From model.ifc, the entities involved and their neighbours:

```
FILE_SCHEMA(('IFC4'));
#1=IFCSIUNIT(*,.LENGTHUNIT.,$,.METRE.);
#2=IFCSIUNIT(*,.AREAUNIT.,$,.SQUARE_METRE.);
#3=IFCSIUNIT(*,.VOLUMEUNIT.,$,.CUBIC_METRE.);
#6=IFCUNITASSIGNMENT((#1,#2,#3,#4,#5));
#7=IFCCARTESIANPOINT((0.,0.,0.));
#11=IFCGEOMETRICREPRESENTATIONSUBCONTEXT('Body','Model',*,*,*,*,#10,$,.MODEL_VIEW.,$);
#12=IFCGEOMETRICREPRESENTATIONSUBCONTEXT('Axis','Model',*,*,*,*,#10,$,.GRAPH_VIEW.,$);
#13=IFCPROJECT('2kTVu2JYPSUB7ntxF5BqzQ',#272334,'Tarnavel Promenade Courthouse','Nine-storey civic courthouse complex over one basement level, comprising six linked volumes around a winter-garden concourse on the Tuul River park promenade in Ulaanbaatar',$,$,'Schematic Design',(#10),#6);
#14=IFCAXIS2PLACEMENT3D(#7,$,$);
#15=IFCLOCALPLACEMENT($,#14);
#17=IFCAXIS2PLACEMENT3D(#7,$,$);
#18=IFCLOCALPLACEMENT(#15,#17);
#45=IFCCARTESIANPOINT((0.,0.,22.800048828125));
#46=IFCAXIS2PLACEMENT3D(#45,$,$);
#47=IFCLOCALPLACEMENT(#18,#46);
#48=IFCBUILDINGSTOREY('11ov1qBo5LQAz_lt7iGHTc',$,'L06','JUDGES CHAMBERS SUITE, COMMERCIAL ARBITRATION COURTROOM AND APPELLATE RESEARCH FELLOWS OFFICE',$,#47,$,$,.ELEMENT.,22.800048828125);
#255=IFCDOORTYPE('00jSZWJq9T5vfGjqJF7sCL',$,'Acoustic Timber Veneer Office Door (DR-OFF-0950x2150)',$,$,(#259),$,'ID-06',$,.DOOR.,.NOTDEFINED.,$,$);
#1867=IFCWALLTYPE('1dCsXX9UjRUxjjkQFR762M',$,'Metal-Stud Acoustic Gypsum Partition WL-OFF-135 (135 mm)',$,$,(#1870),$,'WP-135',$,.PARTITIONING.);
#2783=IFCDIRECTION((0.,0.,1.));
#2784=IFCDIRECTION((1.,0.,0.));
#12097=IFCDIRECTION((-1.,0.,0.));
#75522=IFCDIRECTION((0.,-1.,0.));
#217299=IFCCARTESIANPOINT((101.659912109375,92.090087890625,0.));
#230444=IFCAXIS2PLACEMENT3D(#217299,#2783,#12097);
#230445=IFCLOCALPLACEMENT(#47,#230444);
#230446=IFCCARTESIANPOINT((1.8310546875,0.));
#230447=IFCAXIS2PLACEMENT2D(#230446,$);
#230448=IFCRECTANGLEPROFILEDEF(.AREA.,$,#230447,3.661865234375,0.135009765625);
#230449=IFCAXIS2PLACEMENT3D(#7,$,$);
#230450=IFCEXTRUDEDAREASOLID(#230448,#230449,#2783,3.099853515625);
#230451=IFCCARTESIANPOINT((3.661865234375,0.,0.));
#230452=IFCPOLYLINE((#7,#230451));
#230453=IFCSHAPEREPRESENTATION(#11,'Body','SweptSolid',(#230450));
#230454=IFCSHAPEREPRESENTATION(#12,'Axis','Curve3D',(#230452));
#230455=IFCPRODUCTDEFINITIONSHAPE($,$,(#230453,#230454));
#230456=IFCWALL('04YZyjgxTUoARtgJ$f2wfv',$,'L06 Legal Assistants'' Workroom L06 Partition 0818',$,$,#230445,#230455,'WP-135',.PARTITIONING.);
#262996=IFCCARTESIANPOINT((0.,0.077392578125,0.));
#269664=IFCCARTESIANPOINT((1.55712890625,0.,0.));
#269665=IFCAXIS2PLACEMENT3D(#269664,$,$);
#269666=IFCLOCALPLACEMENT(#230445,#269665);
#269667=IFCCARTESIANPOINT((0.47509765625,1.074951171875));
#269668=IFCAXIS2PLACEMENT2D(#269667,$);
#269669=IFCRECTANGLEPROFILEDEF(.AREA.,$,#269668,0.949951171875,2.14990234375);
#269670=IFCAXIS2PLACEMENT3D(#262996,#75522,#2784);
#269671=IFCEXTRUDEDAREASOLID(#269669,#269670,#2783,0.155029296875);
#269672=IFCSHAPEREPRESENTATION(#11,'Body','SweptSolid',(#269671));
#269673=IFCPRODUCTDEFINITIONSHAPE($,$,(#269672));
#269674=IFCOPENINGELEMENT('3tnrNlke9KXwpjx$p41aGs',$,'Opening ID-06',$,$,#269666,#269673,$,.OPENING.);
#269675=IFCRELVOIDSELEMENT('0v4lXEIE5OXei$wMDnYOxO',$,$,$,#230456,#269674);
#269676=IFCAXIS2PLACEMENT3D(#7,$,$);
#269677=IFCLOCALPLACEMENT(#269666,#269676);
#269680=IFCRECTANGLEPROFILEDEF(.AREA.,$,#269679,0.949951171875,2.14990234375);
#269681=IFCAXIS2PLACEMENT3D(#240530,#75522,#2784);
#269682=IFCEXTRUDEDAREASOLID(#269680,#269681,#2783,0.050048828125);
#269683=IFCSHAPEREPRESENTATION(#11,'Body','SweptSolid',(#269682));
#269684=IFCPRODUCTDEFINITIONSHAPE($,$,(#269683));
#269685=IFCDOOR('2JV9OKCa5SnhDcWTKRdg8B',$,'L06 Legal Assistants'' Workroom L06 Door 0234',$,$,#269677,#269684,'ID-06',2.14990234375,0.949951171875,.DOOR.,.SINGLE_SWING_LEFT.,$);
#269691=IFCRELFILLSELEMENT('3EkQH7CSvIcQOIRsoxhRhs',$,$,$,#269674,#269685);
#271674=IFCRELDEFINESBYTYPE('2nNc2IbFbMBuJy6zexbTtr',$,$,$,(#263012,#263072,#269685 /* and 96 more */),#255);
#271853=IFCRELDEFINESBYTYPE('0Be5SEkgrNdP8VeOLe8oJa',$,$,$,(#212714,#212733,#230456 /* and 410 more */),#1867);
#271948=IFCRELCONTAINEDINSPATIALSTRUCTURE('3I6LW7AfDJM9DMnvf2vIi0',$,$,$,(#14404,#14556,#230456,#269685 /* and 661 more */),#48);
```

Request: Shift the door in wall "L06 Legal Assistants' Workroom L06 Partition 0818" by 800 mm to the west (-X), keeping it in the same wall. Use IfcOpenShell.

```python
import ifcopenshell
import ifcopenshell.api.geometry
import ifcopenshell.util.placement

model = ifcopenshell.open("model.ifc")

door = model.by_guid("2JV9OKCa5SnhDcWTKRdg8B")
opening = door.FillsVoids[0].RelatingOpeningElement
wall = opening.VoidsElements[0].RelatingBuildingElement

wall_matrix = ifcopenshell.util.placement.get_local_placement(wall.ObjectPlacement)
shift = wall_matrix[:3, 0] * 0.8
before = ifcopenshell.util.placement.get_local_placement(door.ObjectPlacement)[:3, 3].copy()

# The door is placed relative to its opening, so it follows when the opening moves.
matrix = ifcopenshell.util.placement.get_local_placement(opening.ObjectPlacement)
matrix[:3, 3] += shift
ifcopenshell.api.geometry.edit_object_placement(
    model, product=opening, matrix=matrix, is_si=False, should_transform_children=True
)

after = ifcopenshell.util.placement.get_local_placement(door.ObjectPlacement)[:3, 3]
print("door moved by", (after - before).round(3) + 0.0)

model.write("model_v2.ifc")
```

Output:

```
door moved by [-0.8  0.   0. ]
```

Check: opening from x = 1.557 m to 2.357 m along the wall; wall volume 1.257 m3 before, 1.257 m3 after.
